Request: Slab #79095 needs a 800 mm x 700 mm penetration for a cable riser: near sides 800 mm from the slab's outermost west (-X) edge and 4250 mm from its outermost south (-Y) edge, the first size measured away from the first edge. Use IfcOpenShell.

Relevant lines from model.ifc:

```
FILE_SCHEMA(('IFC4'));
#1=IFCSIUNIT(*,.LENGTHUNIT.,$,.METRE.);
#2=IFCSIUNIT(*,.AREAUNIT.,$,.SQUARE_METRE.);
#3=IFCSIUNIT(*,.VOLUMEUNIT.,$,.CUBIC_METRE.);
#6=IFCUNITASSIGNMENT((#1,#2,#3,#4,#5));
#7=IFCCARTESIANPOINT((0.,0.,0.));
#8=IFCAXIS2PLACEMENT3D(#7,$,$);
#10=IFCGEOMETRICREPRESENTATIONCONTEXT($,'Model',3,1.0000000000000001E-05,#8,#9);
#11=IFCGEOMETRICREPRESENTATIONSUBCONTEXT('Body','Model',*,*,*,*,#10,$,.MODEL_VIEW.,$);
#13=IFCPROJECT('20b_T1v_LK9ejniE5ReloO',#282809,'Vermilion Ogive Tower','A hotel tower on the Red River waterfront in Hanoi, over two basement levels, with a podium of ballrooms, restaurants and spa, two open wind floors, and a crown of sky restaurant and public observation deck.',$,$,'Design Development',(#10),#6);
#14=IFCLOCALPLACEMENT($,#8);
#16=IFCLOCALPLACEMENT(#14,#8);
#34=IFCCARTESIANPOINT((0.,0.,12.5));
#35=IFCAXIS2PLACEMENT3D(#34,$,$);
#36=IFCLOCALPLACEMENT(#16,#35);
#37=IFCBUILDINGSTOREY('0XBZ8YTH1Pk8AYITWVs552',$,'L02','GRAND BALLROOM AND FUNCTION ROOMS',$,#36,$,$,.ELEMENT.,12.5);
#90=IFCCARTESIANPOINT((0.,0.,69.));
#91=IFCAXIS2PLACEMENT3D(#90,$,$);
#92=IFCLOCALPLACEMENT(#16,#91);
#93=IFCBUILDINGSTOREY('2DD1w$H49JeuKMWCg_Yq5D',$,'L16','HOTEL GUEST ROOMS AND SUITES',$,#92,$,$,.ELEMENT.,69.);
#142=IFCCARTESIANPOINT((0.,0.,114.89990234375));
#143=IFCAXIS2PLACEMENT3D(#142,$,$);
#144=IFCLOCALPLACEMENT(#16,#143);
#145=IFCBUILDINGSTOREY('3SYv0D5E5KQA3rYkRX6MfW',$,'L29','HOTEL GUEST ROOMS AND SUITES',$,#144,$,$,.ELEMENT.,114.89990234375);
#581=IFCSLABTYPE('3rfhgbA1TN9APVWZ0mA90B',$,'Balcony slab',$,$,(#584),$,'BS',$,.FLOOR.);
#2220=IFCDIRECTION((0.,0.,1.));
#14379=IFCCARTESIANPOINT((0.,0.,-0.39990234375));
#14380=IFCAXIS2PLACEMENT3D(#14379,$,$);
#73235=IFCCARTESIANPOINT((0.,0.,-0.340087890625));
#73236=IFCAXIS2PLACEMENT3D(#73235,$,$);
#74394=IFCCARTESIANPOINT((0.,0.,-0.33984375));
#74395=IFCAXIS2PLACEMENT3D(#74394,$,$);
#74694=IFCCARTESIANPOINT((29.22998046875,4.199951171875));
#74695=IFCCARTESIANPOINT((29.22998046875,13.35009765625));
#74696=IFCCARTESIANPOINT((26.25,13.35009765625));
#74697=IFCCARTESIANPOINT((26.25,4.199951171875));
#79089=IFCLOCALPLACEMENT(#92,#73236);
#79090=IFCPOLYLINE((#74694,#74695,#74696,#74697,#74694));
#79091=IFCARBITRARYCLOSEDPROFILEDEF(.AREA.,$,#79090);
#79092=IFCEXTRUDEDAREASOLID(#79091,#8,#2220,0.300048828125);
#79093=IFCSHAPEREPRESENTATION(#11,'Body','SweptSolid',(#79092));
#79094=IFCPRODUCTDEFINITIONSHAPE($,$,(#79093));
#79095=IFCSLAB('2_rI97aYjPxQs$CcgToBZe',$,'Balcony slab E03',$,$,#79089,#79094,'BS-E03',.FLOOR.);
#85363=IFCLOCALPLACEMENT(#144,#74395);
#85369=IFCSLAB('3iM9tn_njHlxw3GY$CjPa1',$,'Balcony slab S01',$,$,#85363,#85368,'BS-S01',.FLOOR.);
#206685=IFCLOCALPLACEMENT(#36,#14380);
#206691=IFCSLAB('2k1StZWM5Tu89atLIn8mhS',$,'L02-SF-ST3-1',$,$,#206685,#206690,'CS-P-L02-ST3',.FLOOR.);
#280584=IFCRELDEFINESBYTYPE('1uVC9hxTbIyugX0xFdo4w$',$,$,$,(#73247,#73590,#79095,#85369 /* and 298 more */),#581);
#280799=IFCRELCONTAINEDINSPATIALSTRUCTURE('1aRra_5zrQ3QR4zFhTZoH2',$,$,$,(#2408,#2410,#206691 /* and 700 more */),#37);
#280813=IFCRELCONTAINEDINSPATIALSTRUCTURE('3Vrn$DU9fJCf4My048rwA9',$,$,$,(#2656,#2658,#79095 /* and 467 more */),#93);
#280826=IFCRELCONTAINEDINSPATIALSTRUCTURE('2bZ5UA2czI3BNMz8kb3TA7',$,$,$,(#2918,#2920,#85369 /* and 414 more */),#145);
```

```python
import numpy as np
import ifcopenshell
import ifcopenshell.api.feature
import ifcopenshell.api.geometry
import ifcopenshell.api.root
import ifcopenshell.geom
import ifcopenshell.util.placement
import ifcopenshell.util.representation
import ifcopenshell.util.shape
import ifcopenshell.util.unit

model = ifcopenshell.open("model.ifc")
unit_scale = ifcopenshell.util.unit.calculate_unit_scale(model)
settings = ifcopenshell.geom.settings()


def volume(element):
    """Net volume in cubic metres, openings subtracted."""
    shape = ifcopenshell.geom.create_shape(settings, element)
    return ifcopenshell.util.shape.get_volume(shape.geometry)


slab = model.by_guid("2_rI97aYjPxQs$CcgToBZe")
before = volume(slab)

# Extent in the slab's own axes, in metres. The edges named are its -X and -Y sides.
slab_shape = ifcopenshell.geom.create_shape(settings, slab)
vertices = ifcopenshell.util.shape.get_vertices(slab_shape.geometry)
x_min, y_min, bottom = vertices.min(axis=0)
top = vertices[:, 2].max()

opening = ifcopenshell.api.root.create_entity(model, ifc_class="IfcOpeningElement", name="Cable riser opening", predefined_type="OPENING")
context = ifcopenshell.util.representation.get_context(model, "Model", "Body", "MODEL_VIEW")
width, depth = 0.8, 0.7
outline = [(0.0, 0.0), (width, 0.0), (width, depth), (0.0, depth), (0.0, 0.0)]
# Overshoot both faces by 50 mm so the cut is clean.
shape = ifcopenshell.api.geometry.add_slab_representation(
    model, context=context, depth=top - bottom + 0.1, polyline=outline
)
ifcopenshell.api.geometry.assign_representation(model, product=opening, representation=shape)

matrix = ifcopenshell.util.placement.get_local_placement(slab.ObjectPlacement)
matrix[:, 3] = matrix @ np.append(np.array([x_min + 0.8, y_min + 4.25, bottom - 0.05]) / unit_scale, 1.0)
ifcopenshell.api.geometry.edit_object_placement(model, product=opening, matrix=matrix, is_si=False)
ifcopenshell.api.feature.add_feature(model, feature=opening, element=slab)

after = volume(slab)

print(f"slab volume {before:.3f} -> {after:.3f} m3")

model.write("model_rev.ifc")
```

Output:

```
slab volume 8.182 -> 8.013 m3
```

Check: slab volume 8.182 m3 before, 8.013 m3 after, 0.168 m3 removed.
